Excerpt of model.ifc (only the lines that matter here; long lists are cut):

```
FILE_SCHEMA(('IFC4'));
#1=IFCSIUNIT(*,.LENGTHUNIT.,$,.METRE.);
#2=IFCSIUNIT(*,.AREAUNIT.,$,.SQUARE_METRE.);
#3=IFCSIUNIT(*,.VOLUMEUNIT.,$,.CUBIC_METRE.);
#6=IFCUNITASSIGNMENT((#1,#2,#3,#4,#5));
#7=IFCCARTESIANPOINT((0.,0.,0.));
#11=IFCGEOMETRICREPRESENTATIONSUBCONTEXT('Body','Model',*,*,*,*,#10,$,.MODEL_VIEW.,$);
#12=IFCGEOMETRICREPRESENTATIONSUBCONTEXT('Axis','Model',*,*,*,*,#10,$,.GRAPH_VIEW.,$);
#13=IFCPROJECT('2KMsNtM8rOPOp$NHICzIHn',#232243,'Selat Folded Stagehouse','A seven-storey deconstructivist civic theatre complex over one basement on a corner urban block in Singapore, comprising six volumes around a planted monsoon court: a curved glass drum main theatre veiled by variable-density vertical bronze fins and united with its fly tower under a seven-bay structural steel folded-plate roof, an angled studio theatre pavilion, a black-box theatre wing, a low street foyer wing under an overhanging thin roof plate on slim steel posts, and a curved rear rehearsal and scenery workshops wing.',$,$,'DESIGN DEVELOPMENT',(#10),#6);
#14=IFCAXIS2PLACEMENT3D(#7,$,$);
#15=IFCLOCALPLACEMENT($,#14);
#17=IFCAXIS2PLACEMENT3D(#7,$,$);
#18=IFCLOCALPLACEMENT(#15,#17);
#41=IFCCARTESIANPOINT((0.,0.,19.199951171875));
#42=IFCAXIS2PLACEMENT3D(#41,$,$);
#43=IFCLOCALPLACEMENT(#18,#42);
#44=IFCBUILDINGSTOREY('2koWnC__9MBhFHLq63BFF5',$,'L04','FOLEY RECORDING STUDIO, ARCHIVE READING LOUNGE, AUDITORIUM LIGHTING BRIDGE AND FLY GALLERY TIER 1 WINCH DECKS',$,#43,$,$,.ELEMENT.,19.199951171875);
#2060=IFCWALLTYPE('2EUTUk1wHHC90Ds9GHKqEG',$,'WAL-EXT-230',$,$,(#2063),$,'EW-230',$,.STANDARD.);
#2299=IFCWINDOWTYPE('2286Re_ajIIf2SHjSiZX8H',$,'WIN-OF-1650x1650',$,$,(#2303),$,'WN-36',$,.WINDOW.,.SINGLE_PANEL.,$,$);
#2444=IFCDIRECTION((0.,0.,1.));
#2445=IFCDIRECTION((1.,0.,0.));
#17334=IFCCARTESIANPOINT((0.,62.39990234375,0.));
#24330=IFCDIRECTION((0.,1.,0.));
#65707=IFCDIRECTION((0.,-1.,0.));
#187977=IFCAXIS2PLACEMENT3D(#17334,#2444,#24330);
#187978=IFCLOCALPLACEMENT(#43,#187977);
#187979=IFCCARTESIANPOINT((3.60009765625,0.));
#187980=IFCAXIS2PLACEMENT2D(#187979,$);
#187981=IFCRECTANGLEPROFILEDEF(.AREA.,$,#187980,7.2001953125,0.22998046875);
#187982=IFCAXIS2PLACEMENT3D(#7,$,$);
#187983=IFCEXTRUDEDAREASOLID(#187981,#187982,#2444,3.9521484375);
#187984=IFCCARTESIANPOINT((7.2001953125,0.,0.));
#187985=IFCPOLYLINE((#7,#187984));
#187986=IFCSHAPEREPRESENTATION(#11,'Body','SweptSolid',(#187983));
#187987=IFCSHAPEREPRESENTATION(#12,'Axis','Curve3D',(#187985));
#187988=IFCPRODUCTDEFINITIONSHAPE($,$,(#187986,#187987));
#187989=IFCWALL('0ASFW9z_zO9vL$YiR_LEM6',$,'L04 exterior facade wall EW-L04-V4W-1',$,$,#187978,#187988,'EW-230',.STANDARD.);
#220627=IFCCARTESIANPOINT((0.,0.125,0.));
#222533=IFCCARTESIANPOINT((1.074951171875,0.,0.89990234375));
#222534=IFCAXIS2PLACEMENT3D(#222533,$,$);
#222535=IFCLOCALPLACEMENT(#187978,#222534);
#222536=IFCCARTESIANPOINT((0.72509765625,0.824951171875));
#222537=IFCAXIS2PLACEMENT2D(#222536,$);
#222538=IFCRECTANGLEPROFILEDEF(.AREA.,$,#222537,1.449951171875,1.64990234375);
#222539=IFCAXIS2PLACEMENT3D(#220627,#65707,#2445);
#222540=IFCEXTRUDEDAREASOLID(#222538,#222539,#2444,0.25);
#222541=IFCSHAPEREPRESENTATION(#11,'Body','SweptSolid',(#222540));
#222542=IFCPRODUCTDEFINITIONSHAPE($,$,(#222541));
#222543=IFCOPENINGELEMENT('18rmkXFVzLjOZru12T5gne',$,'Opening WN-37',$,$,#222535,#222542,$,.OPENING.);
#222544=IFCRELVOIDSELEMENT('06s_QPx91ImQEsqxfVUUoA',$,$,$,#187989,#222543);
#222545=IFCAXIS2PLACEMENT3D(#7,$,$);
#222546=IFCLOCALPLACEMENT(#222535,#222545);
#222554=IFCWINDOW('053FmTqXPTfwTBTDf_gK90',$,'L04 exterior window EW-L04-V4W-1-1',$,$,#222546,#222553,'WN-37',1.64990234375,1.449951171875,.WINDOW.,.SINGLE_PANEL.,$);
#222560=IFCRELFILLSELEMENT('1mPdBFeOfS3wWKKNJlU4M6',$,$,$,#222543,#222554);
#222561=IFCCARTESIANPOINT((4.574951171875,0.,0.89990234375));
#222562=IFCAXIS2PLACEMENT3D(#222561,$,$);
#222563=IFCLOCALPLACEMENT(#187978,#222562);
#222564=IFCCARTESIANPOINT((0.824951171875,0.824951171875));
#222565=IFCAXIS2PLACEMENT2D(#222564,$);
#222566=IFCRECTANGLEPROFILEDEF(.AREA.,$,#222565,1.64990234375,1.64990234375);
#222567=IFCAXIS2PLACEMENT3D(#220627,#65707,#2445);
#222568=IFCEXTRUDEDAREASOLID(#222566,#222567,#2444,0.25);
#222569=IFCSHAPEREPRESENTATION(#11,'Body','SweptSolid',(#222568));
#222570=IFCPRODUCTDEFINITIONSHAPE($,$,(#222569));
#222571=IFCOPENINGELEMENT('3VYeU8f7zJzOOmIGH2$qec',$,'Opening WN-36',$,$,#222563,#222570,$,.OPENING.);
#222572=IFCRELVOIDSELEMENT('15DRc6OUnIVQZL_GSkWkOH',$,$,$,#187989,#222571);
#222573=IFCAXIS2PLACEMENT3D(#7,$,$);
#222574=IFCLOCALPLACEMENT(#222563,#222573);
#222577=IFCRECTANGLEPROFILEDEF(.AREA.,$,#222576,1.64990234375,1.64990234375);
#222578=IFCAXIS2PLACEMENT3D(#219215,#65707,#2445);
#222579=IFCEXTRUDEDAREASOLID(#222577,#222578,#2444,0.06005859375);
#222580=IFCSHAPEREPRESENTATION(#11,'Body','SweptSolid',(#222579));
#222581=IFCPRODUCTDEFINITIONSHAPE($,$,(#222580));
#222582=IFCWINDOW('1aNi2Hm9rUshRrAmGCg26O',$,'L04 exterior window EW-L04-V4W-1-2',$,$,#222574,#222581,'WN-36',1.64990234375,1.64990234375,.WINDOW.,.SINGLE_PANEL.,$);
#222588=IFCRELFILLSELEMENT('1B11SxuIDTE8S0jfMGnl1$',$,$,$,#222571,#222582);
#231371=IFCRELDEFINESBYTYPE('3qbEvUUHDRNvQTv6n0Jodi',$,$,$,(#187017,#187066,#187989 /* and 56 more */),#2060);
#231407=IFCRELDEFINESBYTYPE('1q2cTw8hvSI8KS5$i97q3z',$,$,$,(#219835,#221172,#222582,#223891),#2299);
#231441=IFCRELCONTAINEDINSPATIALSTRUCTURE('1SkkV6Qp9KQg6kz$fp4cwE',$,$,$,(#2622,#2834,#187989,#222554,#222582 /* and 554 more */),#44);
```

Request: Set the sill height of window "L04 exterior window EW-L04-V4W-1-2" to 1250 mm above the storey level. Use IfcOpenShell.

```python
import numpy as np
import ifcopenshell
import ifcopenshell.api.geometry
import ifcopenshell.geom
import ifcopenshell.util.element
import ifcopenshell.util.placement
import ifcopenshell.util.shape
import ifcopenshell.util.unit

model = ifcopenshell.open("model.ifc")
unit_scale = ifcopenshell.util.unit.calculate_unit_scale(model)

window = model.by_guid("1aNi2Hm9rUshRrAmGCg26O")
opening = window.FillsVoids[0].RelatingOpeningElement
storey = ifcopenshell.util.element.get_container(window, ifc_class="IfcBuildingStorey")
level = ifcopenshell.util.placement.get_local_placement(storey.ObjectPlacement)[2, 3]

# The opening's origin need not be at the sill, so measure its lowest point.
shape = ifcopenshell.geom.create_shape(ifcopenshell.geom.settings(), opening)
bottom = ifcopenshell.util.shape.get_shape_bottom_elevation(shape, shape.geometry) / unit_scale
dz = level + 1.25 - bottom

shift = np.array([0.0, 0.0, dz])
# The window is placed relative to its opening, so it follows when the opening moves.
matrix = ifcopenshell.util.placement.get_local_placement(opening.ObjectPlacement)
matrix[:3, 3] += shift
ifcopenshell.api.geometry.edit_object_placement(
    model, product=opening, matrix=matrix, is_si=False, should_transform_children=True
)

print(f"moved by {dz * unit_scale:+.3f} m")

model.write("model_updated.ifc")
```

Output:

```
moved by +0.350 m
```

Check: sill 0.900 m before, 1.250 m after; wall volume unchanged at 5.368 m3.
